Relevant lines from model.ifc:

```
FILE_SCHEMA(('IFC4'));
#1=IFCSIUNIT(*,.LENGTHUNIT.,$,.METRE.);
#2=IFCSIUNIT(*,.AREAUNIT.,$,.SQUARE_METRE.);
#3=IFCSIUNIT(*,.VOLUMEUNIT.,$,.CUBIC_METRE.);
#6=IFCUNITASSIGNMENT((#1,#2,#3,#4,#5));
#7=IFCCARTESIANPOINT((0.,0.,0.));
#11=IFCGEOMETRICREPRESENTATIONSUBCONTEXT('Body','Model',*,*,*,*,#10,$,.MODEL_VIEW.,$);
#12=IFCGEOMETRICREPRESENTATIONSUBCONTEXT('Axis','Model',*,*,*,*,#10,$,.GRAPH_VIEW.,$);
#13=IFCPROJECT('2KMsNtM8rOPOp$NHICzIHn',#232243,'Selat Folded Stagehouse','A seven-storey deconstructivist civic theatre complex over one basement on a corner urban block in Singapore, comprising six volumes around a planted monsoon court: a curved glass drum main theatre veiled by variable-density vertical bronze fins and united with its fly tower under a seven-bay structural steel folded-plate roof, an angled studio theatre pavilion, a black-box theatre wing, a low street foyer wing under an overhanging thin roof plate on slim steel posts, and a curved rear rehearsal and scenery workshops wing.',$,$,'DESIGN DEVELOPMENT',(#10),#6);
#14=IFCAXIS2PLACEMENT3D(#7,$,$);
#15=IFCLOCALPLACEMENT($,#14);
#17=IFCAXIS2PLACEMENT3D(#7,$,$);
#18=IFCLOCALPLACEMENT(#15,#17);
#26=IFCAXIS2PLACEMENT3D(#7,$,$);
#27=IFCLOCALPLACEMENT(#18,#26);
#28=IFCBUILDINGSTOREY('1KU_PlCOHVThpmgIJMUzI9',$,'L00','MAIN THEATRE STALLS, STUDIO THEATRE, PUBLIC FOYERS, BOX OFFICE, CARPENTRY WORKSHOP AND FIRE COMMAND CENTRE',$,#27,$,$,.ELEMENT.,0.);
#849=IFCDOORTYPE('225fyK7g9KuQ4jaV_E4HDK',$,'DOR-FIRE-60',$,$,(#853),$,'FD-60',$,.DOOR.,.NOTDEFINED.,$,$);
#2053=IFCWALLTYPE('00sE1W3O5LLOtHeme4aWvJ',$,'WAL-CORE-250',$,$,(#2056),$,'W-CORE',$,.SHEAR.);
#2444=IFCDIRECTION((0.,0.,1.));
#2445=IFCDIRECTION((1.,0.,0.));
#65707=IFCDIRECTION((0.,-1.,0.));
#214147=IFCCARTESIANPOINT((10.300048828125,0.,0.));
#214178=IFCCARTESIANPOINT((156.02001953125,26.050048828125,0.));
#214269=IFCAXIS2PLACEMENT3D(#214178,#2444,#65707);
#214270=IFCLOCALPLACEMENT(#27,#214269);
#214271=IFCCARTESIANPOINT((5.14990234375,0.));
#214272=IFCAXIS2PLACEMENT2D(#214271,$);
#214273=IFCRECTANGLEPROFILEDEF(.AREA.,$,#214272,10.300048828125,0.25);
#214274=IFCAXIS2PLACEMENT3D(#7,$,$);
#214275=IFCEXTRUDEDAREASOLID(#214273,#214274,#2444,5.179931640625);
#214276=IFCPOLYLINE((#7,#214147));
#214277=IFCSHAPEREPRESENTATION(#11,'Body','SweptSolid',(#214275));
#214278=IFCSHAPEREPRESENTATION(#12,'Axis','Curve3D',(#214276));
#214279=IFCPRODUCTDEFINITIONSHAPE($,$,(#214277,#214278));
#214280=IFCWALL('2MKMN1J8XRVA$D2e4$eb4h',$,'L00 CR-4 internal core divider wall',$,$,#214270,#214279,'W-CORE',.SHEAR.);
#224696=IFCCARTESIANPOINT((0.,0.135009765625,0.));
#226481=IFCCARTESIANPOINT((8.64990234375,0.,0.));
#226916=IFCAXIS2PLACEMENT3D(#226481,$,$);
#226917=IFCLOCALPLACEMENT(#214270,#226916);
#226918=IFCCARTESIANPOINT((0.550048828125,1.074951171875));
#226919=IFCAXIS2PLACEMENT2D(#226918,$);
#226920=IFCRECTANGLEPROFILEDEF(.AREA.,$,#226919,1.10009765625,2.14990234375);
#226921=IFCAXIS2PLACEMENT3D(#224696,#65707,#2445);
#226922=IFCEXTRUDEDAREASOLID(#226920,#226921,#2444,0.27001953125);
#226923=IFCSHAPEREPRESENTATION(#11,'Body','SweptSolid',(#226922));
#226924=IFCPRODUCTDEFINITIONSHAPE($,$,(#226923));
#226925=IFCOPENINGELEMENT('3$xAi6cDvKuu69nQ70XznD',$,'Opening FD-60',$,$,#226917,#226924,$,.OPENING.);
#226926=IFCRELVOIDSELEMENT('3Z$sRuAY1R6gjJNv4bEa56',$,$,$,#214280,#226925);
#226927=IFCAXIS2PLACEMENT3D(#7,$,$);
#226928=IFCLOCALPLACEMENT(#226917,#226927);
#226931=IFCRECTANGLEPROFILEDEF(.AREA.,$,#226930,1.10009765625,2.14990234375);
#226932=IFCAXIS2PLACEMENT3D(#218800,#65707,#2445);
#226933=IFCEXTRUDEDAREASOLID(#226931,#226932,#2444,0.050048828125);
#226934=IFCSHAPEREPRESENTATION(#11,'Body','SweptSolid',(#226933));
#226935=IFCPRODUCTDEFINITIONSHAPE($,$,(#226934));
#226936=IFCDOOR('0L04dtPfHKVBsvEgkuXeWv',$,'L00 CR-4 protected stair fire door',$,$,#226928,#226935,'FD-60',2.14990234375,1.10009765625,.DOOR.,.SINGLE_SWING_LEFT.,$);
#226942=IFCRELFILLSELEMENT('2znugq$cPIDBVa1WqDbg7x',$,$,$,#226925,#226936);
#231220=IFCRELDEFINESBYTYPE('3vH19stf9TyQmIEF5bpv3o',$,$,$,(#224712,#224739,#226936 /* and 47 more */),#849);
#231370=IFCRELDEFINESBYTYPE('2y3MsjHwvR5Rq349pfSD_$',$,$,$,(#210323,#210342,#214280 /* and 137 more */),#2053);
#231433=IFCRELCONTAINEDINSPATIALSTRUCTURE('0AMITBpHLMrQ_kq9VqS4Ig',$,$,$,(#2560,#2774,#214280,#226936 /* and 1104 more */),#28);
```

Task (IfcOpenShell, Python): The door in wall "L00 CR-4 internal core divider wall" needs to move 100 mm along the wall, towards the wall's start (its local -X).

```python
import ifcopenshell
import ifcopenshell.api.geometry
import ifcopenshell.util.placement

model = ifcopenshell.open("model.ifc")

door = model.by_guid("0L04dtPfHKVBsvEgkuXeWv")
opening = door.FillsVoids[0].RelatingOpeningElement
wall = opening.VoidsElements[0].RelatingBuildingElement

wall_matrix = ifcopenshell.util.placement.get_local_placement(wall.ObjectPlacement)
shift = wall_matrix[:3, 0] * -0.1
before = ifcopenshell.util.placement.get_local_placement(door.ObjectPlacement)[:3, 3].copy()

# The door is placed relative to its opening, so it follows when the opening moves.
matrix = ifcopenshell.util.placement.get_local_placement(opening.ObjectPlacement)
matrix[:3, 3] += shift
ifcopenshell.api.geometry.edit_object_placement(
    model, product=opening, matrix=matrix, is_si=False, should_transform_children=True
)

after = ifcopenshell.util.placement.get_local_placement(door.ObjectPlacement)[:3, 3]
print("door moved by", (after - before).round(3) + 0.0)

model.write("model_rev.ifc")
```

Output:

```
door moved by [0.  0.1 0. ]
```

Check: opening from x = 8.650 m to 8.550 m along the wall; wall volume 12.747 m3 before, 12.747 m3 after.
